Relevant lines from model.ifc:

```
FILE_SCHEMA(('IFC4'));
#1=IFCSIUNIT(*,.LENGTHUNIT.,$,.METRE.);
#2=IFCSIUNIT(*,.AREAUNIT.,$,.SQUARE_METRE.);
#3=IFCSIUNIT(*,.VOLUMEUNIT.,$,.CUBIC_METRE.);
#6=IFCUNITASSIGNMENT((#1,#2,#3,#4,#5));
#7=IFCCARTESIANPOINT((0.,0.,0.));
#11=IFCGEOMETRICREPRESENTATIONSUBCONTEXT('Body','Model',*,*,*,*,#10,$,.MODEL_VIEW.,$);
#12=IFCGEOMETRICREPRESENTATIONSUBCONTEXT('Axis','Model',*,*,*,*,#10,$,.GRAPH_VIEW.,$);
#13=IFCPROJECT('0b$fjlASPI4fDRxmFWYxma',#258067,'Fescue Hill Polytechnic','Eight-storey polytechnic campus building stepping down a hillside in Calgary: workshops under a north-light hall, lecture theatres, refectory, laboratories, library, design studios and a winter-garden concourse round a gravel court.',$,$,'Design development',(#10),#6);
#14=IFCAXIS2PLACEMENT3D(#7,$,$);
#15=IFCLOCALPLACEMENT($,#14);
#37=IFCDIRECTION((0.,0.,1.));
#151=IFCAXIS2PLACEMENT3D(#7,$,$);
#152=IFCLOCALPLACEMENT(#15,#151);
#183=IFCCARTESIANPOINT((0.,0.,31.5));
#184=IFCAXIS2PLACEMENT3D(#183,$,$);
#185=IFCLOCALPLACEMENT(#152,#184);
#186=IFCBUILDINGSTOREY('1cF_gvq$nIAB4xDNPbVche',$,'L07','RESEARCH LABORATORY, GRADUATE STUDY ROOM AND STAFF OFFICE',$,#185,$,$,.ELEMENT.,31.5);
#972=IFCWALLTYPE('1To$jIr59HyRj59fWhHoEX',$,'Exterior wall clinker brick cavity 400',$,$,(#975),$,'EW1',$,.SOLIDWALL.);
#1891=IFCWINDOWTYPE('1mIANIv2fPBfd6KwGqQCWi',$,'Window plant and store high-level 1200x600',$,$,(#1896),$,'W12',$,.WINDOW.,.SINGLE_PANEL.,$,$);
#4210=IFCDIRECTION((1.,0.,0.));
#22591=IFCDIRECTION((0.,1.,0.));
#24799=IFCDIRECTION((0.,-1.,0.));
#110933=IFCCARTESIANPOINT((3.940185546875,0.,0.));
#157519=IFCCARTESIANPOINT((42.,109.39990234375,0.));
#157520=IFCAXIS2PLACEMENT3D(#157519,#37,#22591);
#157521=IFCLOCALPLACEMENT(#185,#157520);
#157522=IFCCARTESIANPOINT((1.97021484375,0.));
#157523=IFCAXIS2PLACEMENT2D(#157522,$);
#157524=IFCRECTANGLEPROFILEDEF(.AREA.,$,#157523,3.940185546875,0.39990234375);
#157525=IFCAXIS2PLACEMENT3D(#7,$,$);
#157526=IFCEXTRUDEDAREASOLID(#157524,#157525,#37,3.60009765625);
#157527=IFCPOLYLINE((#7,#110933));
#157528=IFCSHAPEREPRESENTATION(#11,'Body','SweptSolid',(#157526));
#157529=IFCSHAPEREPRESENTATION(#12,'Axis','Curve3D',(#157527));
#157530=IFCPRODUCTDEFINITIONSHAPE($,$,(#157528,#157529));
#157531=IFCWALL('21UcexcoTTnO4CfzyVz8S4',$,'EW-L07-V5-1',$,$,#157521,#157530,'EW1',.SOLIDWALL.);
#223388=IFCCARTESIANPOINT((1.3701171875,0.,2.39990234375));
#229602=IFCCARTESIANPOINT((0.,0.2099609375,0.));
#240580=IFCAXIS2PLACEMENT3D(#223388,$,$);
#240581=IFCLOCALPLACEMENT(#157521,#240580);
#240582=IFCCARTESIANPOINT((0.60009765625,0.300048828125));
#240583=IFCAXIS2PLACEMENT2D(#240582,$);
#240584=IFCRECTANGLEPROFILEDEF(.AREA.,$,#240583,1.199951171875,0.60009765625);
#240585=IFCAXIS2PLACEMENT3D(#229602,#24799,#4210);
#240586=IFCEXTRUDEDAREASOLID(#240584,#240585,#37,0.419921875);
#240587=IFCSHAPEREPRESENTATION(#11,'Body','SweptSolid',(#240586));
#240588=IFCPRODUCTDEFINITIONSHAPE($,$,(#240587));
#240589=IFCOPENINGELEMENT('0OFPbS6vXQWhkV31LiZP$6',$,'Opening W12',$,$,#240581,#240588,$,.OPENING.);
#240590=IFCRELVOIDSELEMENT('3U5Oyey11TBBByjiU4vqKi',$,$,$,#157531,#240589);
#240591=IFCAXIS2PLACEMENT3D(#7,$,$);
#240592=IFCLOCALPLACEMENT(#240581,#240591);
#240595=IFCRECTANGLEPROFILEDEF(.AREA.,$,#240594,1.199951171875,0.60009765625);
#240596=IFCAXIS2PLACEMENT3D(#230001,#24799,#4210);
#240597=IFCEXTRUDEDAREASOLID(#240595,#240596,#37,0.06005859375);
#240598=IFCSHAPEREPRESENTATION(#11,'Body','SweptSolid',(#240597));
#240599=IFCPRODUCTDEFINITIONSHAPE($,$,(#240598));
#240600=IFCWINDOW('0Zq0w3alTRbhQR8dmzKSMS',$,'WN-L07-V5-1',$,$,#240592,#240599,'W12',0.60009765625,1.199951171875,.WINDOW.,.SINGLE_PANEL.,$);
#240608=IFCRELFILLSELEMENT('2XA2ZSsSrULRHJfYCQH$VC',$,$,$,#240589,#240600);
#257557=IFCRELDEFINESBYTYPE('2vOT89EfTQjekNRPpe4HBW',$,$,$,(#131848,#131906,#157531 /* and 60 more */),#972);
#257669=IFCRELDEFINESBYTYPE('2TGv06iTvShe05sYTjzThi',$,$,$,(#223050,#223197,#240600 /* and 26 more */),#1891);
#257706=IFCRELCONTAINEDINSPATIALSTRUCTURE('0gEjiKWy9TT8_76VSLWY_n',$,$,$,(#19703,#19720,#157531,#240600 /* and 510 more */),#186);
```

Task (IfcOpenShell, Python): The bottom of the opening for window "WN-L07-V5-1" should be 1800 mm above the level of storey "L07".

```python
import numpy as np
import ifcopenshell
import ifcopenshell.api.geometry
import ifcopenshell.geom
import ifcopenshell.util.element
import ifcopenshell.util.placement
import ifcopenshell.util.shape
import ifcopenshell.util.unit

model = ifcopenshell.open("model.ifc")
unit_scale = ifcopenshell.util.unit.calculate_unit_scale(model)

window = model.by_guid("0Zq0w3alTRbhQR8dmzKSMS")
opening = window.FillsVoids[0].RelatingOpeningElement
storey = ifcopenshell.util.element.get_container(window, ifc_class="IfcBuildingStorey")
level = ifcopenshell.util.placement.get_local_placement(storey.ObjectPlacement)[2, 3]

# The opening's origin need not be at the sill, so measure its lowest point.
shape = ifcopenshell.geom.create_shape(ifcopenshell.geom.settings(), opening)
bottom = ifcopenshell.util.shape.get_shape_bottom_elevation(shape, shape.geometry) / unit_scale
dz = level + 1.8 - bottom

shift = np.array([0.0, 0.0, dz])
# The window is placed relative to its opening, so it follows when the opening moves.
matrix = ifcopenshell.util.placement.get_local_placement(opening.ObjectPlacement)
matrix[:3, 3] += shift
ifcopenshell.api.geometry.edit_object_placement(
    model, product=opening, matrix=matrix, is_si=False, should_transform_children=True
)

print(f"moved by {dz * unit_scale:+.3f} m")

model.write("model_updated.ifc")
```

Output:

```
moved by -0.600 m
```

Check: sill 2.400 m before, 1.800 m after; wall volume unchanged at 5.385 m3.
